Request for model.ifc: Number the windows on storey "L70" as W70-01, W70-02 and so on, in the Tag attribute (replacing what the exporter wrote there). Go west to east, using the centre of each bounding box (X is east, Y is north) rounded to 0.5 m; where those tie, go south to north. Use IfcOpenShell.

First a look at what the model holds.

```python
import ifcopenshell
import ifcopenshell.util.element
import ifcopenshell.util.placement

model = ifcopenshell.open("model.ifc")
print(model.schema)
storey = next(s for s in model.by_type("IfcBuildingStorey") if s.Name == "L70")
windows = [e for e in ifcopenshell.util.element.get_decomposition(storey) if e.is_a("IfcWindow")]
for e in sorted(windows, key=lambda e: e.id()):
    origin = ifcopenshell.util.placement.get_local_placement(e.ObjectPlacement)[:3, 3]
    print(e.id(), e.Tag, e.Name, origin.round(2) + 0.0, sep=" | ")
```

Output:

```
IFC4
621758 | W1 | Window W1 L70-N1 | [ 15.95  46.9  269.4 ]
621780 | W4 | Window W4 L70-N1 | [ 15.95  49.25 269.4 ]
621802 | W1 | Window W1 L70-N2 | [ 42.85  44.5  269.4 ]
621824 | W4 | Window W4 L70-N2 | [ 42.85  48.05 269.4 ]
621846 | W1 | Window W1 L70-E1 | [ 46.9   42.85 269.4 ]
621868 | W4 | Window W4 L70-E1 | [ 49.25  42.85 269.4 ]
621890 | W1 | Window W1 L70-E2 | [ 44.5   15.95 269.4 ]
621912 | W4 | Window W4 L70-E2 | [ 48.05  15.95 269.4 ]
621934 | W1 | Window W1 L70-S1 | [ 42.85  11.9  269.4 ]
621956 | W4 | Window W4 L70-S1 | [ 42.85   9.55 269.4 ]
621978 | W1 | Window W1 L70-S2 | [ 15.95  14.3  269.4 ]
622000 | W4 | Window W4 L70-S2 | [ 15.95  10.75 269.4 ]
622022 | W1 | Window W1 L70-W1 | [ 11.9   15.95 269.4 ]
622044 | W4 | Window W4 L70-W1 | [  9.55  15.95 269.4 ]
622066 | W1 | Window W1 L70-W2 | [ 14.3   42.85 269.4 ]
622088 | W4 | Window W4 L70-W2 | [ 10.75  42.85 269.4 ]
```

```python
import ifcopenshell
import ifcopenshell.geom
import ifcopenshell.util.element
import ifcopenshell.util.shape

model = ifcopenshell.open("model.ifc")
settings = ifcopenshell.geom.settings()
settings.set("use-world-coords", True)


def centre(element):
    shape = ifcopenshell.geom.create_shape(settings, element)
    return ifcopenshell.util.shape.get_bbox_centroid(shape.geometry)


storey = next(s for s in model.by_type("IfcBuildingStorey") if s.Name == "L70")
windows = [e for e in ifcopenshell.util.element.get_decomposition(storey) if e.is_a("IfcWindow")]

# Insertion points can sit at a corner or the storey origin, so sort by the geometry (in metres).
centres = {e: centre(e) for e in windows}
windows.sort(key=lambda e: (round(centres[e][0] / 0.5), centres[e][1]))

for i, e in enumerate(windows, start=1):
    number = f"W70-{i:02d}"
    e.Tag = number
    print(e.id(), number)

model.write("model_edited.ifc")
```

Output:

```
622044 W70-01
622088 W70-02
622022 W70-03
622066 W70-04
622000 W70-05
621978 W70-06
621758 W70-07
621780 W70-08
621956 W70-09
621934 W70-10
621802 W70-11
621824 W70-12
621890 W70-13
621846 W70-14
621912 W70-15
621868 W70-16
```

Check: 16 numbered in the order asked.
